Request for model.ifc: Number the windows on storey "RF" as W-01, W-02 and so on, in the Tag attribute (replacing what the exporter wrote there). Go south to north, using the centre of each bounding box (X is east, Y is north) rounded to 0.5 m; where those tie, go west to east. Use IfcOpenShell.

First a look at what the model holds.

```python
import ifcopenshell
import ifcopenshell.util.element
import ifcopenshell.util.placement

model = ifcopenshell.open("model.ifc")
print(model.schema)
storey = next(s for s in model.by_type("IfcBuildingStorey") if s.Name == "RF")
windows = [e for e in ifcopenshell.util.element.get_decomposition(storey) if e.is_a("IfcWindow")]
for e in sorted(windows, key=lambda e: e.id()):
    origin = ifcopenshell.util.placement.get_local_placement(e.ObjectPlacement)[:3, 3]
    print(e.id(), e.Tag, e.Name, origin.round(2) + 0.0, sep=" | ")
```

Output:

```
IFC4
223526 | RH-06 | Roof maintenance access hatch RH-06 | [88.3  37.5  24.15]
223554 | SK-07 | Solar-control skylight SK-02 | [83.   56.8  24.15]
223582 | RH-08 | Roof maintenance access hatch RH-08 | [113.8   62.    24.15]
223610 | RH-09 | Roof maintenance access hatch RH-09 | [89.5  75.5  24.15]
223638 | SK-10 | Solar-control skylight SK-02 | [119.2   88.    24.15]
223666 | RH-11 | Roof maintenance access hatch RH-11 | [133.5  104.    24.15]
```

```python
import ifcopenshell
import ifcopenshell.geom
import ifcopenshell.util.element
import ifcopenshell.util.shape

model = ifcopenshell.open("model.ifc")
settings = ifcopenshell.geom.settings()
settings.set("use-world-coords", True)


def centre(element):
    shape = ifcopenshell.geom.create_shape(settings, element)
    return ifcopenshell.util.shape.get_bbox_centroid(shape.geometry)


storey = next(s for s in model.by_type("IfcBuildingStorey") if s.Name == "RF")
windows = [e for e in ifcopenshell.util.element.get_decomposition(storey) if e.is_a("IfcWindow")]

# Insertion points can sit at a corner or the storey origin, so sort by the geometry (in metres).
centres = {e: centre(e) for e in windows}
windows.sort(key=lambda e: (round(centres[e][1] / 0.5), centres[e][0]))

for i, e in enumerate(windows, start=1):
    number = f"W-{i:02d}"
    e.Tag = number
    print(e.id(), number)

model.write("model_edited.ifc")
```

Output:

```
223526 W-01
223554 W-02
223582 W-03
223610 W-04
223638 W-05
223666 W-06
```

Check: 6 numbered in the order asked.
